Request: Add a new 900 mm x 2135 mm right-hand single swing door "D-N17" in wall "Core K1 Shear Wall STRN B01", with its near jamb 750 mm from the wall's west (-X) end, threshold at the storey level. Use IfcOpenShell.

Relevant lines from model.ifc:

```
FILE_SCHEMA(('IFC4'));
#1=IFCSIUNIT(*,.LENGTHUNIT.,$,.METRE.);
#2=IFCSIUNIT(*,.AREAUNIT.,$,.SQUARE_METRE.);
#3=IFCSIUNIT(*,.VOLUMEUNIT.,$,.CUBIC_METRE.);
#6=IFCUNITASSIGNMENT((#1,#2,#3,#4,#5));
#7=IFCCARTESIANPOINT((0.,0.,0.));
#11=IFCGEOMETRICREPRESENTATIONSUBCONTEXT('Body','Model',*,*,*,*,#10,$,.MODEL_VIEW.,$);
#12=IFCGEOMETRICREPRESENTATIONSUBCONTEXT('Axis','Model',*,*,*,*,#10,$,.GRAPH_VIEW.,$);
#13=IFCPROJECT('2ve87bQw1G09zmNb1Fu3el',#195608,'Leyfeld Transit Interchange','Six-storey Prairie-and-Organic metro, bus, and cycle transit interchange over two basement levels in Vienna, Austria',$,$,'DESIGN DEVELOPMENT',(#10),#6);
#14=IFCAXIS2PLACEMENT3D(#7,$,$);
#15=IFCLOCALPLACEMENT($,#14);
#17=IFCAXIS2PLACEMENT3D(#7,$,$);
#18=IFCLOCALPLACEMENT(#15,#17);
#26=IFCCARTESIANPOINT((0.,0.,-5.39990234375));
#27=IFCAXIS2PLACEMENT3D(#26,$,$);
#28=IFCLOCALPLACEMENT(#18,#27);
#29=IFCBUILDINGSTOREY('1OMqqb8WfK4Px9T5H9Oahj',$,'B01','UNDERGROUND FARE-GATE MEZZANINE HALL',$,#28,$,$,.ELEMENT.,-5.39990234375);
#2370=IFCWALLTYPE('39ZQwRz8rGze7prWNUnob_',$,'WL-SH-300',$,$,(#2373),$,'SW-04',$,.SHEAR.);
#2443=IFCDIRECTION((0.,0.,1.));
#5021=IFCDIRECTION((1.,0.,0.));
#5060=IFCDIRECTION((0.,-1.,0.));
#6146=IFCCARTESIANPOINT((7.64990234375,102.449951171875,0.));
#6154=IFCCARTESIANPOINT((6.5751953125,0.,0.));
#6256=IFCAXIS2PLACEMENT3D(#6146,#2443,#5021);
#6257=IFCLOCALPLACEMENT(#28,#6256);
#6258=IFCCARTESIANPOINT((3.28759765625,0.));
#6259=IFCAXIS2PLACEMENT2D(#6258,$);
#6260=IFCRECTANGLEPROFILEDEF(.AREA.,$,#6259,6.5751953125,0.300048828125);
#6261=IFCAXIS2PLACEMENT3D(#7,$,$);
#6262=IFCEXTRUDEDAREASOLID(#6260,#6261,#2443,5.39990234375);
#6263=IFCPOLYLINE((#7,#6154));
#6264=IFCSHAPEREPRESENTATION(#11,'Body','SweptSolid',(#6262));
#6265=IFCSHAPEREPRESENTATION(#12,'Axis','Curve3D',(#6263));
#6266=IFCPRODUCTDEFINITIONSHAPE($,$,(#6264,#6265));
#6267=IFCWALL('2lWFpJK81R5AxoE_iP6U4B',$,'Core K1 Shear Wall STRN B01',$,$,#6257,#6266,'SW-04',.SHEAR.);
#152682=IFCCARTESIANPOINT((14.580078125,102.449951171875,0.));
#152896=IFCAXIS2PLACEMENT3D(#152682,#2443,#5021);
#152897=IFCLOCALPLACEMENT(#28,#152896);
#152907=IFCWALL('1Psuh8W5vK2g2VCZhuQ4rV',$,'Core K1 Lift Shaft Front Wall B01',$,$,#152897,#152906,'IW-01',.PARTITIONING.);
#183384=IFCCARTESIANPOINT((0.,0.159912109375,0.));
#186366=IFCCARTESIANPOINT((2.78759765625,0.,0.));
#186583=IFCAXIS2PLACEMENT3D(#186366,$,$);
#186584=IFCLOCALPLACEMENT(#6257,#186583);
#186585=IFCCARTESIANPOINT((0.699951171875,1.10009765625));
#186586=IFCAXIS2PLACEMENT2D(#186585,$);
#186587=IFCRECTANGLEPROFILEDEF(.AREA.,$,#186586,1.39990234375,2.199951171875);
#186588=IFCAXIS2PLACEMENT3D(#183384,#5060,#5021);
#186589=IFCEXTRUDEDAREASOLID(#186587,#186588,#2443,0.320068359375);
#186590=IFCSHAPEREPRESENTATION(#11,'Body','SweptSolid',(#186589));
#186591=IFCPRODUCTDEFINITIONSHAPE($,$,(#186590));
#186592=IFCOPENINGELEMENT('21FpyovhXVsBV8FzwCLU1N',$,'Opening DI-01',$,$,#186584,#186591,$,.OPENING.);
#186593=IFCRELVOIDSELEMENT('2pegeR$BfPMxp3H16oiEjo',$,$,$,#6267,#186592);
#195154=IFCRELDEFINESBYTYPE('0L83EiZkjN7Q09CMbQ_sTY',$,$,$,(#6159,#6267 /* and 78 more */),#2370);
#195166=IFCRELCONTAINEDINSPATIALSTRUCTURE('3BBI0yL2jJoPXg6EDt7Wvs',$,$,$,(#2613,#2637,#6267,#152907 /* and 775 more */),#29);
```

```python
import numpy as np
import ifcopenshell
import ifcopenshell.api.feature
import ifcopenshell.api.geometry
import ifcopenshell.api.root
import ifcopenshell.api.spatial
import ifcopenshell.geom
import ifcopenshell.util.element
import ifcopenshell.util.placement
import ifcopenshell.util.representation
import ifcopenshell.util.shape
import ifcopenshell.util.unit

model = ifcopenshell.open("model.ifc")
unit_scale = ifcopenshell.util.unit.calculate_unit_scale(model)
settings = ifcopenshell.geom.settings()


def volume(element):
    """Net volume in cubic metres, openings subtracted."""
    shape = ifcopenshell.geom.create_shape(settings, element)
    return ifcopenshell.util.shape.get_volume(shape.geometry)


wall = model.by_id(6267)
storey = ifcopenshell.util.element.get_container(wall, ifc_class="IfcBuildingStorey")
context = ifcopenshell.util.representation.get_context(model, "Model", "Body", "MODEL_VIEW")
before = volume(wall)

width, height, from_end, sill = 0.9, 2.135, 0.75, 0.0  # metres

# The wall runs along its own X axis, and the end named is its -X end.
wall_shape = ifcopenshell.geom.create_shape(settings, wall)
x, y, z = ifcopenshell.util.shape.get_vertices(wall_shape.geometry).T
start = x.min() + from_end
face, thickness = float(y.min()), float(y.max() - y.min())
wall_matrix = ifcopenshell.util.placement.get_local_placement(wall.ObjectPlacement)
level = ifcopenshell.util.placement.get_local_placement(storey.ObjectPlacement)[2, 3]


def in_wall(x, y):
    """Placement at x, y metres in the wall's axes, at sill height."""
    matrix = wall_matrix.copy()
    matrix[:, 3] = wall_matrix @ np.array([x / unit_scale, y / unit_scale, 0.0, 1.0])
    matrix[2, 3] = level + sill / unit_scale
    return matrix


# Opening: a box that overshoots both wall faces by 50 mm.
opening = ifcopenshell.api.root.create_entity(model, ifc_class="IfcOpeningElement", predefined_type="OPENING")
box = ifcopenshell.api.geometry.add_wall_representation(
    model, context=context, length=width, height=height, thickness=thickness + 0.1
)
ifcopenshell.api.geometry.assign_representation(model, product=opening, representation=box)
ifcopenshell.api.geometry.edit_object_placement(model, product=opening, matrix=in_wall(start, face - 0.05), is_si=False)
ifcopenshell.api.feature.add_feature(model, feature=opening, element=wall)

door = ifcopenshell.api.root.create_entity(model, ifc_class="IfcDoor", name="D-N17", predefined_type="DOOR")
door.OverallWidth, door.OverallHeight = width / unit_scale, height / unit_scale
door.OperationType = "SINGLE_SWING_RIGHT"
body = ifcopenshell.api.geometry.add_door_representation(
    model,
    context=context,
    overall_width=door.OverallWidth,
    overall_height=door.OverallHeight,
    operation_type="SINGLE_SWING_RIGHT",
    lining_properties={"LiningDepth": thickness / unit_scale, "ThresholdDepth": thickness / unit_scale},
)
ifcopenshell.api.geometry.assign_representation(model, product=door, representation=body)
ifcopenshell.api.spatial.assign_container(model, products=[door], relating_structure=storey)
ifcopenshell.api.feature.add_filling(model, opening=opening, element=door)

# The lining spans the wall, so the door starts at the wall face.
ifcopenshell.api.geometry.edit_object_placement(model, product=door, matrix=in_wall(start, face), is_si=False)

after = volume(wall)

print(f"wall volume {before:.3f} -> {after:.3f} m3")

model.write("model-out.ifc")
```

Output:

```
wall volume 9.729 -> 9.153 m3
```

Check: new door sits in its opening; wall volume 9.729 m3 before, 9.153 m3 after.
